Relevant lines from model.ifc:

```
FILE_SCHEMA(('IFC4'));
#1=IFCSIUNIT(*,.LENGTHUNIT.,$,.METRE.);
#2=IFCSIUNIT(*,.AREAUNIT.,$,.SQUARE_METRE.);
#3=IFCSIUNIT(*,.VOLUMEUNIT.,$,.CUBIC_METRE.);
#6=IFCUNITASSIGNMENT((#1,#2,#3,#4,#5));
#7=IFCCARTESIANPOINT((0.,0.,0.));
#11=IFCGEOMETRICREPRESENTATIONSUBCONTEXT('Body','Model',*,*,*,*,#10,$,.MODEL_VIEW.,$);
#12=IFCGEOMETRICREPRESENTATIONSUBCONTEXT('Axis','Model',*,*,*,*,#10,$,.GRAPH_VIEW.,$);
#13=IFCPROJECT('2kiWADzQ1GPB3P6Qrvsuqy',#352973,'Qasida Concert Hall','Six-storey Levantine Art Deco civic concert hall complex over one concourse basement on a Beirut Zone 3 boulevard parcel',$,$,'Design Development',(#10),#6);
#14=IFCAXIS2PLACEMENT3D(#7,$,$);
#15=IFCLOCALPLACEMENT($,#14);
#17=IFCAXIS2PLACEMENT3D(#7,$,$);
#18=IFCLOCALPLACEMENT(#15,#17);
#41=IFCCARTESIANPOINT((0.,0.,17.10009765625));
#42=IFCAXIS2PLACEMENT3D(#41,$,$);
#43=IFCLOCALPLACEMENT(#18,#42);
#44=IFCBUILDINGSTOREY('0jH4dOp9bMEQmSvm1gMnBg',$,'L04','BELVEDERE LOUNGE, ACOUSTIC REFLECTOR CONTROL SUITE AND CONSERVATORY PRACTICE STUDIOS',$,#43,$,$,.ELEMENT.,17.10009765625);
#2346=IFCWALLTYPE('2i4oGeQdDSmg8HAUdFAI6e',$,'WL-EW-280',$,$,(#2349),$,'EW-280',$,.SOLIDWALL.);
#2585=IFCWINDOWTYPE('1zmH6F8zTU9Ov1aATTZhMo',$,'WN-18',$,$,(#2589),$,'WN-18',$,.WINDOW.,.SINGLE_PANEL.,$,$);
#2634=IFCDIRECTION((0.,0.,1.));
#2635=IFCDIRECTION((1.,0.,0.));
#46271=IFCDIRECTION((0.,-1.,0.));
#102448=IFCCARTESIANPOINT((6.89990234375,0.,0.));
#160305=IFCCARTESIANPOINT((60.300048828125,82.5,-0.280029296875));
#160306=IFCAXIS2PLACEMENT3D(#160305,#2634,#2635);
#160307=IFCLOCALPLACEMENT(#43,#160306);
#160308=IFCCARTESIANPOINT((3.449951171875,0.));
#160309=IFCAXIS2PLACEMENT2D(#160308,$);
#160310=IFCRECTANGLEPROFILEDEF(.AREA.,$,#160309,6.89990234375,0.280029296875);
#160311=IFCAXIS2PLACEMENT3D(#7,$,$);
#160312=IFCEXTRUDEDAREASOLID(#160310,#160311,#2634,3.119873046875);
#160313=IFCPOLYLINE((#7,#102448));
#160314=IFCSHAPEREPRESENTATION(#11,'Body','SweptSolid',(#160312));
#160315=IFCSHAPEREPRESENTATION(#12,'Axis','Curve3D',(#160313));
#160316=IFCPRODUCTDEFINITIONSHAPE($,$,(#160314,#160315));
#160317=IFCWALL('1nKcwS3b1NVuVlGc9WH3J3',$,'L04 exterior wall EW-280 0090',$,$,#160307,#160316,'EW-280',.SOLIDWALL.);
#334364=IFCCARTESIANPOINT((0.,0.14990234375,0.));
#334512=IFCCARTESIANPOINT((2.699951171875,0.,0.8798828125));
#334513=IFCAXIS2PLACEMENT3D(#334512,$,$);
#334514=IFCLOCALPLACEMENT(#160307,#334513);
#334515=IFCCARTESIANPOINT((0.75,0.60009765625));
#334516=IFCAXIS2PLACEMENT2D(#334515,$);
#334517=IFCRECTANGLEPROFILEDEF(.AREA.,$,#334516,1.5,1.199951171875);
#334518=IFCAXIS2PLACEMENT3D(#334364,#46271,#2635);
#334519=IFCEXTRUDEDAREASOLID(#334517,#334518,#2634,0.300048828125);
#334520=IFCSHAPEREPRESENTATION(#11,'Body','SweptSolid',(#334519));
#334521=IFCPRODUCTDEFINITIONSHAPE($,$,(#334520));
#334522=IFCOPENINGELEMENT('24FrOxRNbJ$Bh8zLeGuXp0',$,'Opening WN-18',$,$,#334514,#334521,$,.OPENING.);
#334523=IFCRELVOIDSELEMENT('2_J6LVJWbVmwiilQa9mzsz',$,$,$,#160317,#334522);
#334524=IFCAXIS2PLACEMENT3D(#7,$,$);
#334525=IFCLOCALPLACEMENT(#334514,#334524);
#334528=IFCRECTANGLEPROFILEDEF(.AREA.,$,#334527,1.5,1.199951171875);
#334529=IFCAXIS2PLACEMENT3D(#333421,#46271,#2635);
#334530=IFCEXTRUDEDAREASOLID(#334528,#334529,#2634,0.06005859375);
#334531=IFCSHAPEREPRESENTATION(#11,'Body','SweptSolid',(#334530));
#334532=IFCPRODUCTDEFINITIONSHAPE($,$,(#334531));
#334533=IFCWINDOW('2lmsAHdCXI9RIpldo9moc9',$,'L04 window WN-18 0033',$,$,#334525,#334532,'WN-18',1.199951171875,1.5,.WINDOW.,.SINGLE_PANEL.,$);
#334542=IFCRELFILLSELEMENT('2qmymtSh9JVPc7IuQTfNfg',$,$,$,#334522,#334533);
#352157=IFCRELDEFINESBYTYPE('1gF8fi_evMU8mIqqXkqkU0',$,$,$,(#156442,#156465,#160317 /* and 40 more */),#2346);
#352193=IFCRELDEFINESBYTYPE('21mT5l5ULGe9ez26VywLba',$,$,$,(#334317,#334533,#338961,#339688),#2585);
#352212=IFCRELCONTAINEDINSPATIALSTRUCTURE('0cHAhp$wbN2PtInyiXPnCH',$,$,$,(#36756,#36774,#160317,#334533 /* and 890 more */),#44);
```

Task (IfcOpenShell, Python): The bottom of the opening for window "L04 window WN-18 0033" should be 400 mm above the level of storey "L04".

```python
import numpy as np
import ifcopenshell
import ifcopenshell.api.geometry
import ifcopenshell.geom
import ifcopenshell.util.element
import ifcopenshell.util.placement
import ifcopenshell.util.shape
import ifcopenshell.util.unit

model = ifcopenshell.open("model.ifc")
unit_scale = ifcopenshell.util.unit.calculate_unit_scale(model)

window = model.by_id(334533)
opening = window.FillsVoids[0].RelatingOpeningElement
storey = ifcopenshell.util.element.get_container(window, ifc_class="IfcBuildingStorey")
level = ifcopenshell.util.placement.get_local_placement(storey.ObjectPlacement)[2, 3]

# The opening's origin need not be at the sill, so measure its lowest point.
shape = ifcopenshell.geom.create_shape(ifcopenshell.geom.settings(), opening)
bottom = ifcopenshell.util.shape.get_shape_bottom_elevation(shape, shape.geometry) / unit_scale
dz = level + 0.4 - bottom

shift = np.array([0.0, 0.0, dz])
# The window is placed relative to its opening, so it follows when the opening moves.
matrix = ifcopenshell.util.placement.get_local_placement(opening.ObjectPlacement)
matrix[:3, 3] += shift
ifcopenshell.api.geometry.edit_object_placement(
    model, product=opening, matrix=matrix, is_si=False, should_transform_children=True
)

print(f"moved by {dz * unit_scale:+.3f} m")

model.write("model-out.ifc")
```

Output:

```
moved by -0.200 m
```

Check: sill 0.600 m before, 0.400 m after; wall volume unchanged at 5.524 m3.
